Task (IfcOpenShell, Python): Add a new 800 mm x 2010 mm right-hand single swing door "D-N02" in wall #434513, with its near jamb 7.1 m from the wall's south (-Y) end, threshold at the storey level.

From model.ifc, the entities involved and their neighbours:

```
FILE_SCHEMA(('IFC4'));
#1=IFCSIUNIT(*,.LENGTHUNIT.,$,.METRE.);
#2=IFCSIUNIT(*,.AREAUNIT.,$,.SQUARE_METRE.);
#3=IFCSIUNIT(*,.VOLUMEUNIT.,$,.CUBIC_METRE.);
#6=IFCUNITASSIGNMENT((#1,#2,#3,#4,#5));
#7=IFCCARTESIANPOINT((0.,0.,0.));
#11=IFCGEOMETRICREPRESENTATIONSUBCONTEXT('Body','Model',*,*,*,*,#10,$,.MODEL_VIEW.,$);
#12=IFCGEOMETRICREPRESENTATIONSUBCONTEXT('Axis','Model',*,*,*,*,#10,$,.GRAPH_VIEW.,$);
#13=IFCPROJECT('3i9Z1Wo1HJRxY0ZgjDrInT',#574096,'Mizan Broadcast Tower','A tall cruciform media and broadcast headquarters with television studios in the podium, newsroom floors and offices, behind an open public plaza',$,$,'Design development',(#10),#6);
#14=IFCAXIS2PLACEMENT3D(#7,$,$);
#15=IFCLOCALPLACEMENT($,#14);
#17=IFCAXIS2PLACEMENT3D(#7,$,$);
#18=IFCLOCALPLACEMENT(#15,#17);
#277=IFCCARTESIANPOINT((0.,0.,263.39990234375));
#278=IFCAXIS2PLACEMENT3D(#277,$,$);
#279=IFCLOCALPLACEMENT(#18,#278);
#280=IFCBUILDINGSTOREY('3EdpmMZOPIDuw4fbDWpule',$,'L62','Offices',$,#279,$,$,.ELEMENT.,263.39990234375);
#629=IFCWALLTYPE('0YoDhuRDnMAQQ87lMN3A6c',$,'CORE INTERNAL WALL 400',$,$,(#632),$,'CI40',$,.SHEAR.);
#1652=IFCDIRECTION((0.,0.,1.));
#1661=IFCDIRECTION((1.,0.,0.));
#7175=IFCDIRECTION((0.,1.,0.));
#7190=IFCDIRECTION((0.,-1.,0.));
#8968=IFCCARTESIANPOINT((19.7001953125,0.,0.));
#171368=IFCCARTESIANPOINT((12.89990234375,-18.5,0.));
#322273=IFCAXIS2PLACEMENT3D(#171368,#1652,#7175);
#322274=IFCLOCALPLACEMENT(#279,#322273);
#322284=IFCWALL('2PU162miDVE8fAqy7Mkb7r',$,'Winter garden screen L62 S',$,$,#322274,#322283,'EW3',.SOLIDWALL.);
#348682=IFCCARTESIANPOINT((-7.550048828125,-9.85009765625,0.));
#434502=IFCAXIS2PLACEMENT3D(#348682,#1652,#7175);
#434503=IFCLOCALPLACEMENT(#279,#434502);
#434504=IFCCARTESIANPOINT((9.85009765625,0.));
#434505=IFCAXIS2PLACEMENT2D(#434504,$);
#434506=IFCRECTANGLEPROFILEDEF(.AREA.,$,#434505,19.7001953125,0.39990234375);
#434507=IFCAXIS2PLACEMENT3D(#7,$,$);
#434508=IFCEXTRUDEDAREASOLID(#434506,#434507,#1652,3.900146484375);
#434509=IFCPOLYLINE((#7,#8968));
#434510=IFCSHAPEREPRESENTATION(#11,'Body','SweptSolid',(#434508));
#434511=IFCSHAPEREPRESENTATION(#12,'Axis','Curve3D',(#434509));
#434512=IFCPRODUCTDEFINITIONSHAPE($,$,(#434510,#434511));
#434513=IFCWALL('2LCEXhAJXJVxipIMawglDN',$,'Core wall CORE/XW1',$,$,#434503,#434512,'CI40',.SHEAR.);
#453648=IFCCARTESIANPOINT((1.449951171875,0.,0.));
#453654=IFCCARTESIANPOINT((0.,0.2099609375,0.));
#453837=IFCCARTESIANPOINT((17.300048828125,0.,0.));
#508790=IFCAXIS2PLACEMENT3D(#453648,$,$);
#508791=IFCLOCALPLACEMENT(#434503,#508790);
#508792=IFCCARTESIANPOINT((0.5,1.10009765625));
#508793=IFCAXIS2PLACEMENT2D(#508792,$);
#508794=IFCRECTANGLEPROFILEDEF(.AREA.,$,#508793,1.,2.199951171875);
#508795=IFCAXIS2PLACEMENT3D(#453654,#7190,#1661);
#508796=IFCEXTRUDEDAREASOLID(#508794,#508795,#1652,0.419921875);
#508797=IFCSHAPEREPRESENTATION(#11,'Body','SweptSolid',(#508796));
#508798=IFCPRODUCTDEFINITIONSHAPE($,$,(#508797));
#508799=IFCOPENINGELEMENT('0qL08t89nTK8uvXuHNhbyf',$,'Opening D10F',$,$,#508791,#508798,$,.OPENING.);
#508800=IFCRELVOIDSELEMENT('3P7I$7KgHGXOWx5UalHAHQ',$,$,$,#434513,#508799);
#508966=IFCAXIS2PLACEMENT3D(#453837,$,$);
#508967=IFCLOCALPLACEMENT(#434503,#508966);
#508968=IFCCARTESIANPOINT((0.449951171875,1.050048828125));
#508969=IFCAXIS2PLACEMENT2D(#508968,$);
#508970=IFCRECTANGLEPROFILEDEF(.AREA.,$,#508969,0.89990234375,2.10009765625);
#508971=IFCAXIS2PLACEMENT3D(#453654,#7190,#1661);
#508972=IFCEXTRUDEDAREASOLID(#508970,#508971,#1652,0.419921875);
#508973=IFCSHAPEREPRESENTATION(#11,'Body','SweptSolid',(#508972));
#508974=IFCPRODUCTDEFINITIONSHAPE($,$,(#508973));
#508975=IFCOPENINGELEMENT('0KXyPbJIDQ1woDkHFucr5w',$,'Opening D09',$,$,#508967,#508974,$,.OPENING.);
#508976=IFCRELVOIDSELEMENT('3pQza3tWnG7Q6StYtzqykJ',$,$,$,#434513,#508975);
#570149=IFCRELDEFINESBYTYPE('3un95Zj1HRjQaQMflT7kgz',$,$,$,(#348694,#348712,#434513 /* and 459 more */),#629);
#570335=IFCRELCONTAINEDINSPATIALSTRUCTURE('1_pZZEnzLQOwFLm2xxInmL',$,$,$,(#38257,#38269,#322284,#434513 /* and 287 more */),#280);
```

```python
import numpy as np
import ifcopenshell
import ifcopenshell.api.feature
import ifcopenshell.api.geometry
import ifcopenshell.api.root
import ifcopenshell.api.spatial
import ifcopenshell.geom
import ifcopenshell.util.element
import ifcopenshell.util.placement
import ifcopenshell.util.representation
import ifcopenshell.util.shape
import ifcopenshell.util.unit

model = ifcopenshell.open("model.ifc")
unit_scale = ifcopenshell.util.unit.calculate_unit_scale(model)
settings = ifcopenshell.geom.settings()


def volume(element):
    """Net volume in cubic metres, openings subtracted."""
    shape = ifcopenshell.geom.create_shape(settings, element)
    return ifcopenshell.util.shape.get_volume(shape.geometry)


wall = model.by_guid("2LCEXhAJXJVxipIMawglDN")
storey = ifcopenshell.util.element.get_container(wall, ifc_class="IfcBuildingStorey")
context = ifcopenshell.util.representation.get_context(model, "Model", "Body", "MODEL_VIEW")
before = volume(wall)

width, height, from_end, sill = 0.8, 2.01, 7.1, 0.0  # metres

# The wall runs along its own X axis, and the end named is its -X end.
wall_shape = ifcopenshell.geom.create_shape(settings, wall)
x, y, z = ifcopenshell.util.shape.get_vertices(wall_shape.geometry).T
start = x.min() + from_end
face, thickness = float(y.min()), float(y.max() - y.min())
wall_matrix = ifcopenshell.util.placement.get_local_placement(wall.ObjectPlacement)
level = ifcopenshell.util.placement.get_local_placement(storey.ObjectPlacement)[2, 3]


def in_wall(x, y):
    """Placement at x, y metres in the wall's axes, at sill height."""
    matrix = wall_matrix.copy()
    matrix[:, 3] = wall_matrix @ np.array([x / unit_scale, y / unit_scale, 0.0, 1.0])
    matrix[2, 3] = level + sill / unit_scale
    return matrix


# Opening: a box that overshoots both wall faces by 50 mm.
opening = ifcopenshell.api.root.create_entity(model, ifc_class="IfcOpeningElement", predefined_type="OPENING")
box = ifcopenshell.api.geometry.add_wall_representation(
    model, context=context, length=width, height=height, thickness=thickness + 0.1
)
ifcopenshell.api.geometry.assign_representation(model, product=opening, representation=box)
ifcopenshell.api.geometry.edit_object_placement(model, product=opening, matrix=in_wall(start, face - 0.05), is_si=False)
ifcopenshell.api.feature.add_feature(model, feature=opening, element=wall)

door = ifcopenshell.api.root.create_entity(model, ifc_class="IfcDoor", name="D-N02", predefined_type="DOOR")
door.OverallWidth, door.OverallHeight = width / unit_scale, height / unit_scale
door.OperationType = "SINGLE_SWING_RIGHT"
body = ifcopenshell.api.geometry.add_door_representation(
    model,
    context=context,
    overall_width=door.OverallWidth,
    overall_height=door.OverallHeight,
    operation_type="SINGLE_SWING_RIGHT",
    lining_properties={"LiningDepth": thickness / unit_scale, "ThresholdDepth": thickness / unit_scale},
)
ifcopenshell.api.geometry.assign_representation(model, product=door, representation=body)
ifcopenshell.api.spatial.assign_container(model, products=[door], relating_structure=storey)
ifcopenshell.api.feature.add_filling(model, opening=opening, element=door)

# The lining spans the wall, so the door starts at the wall face.
ifcopenshell.api.geometry.edit_object_placement(model, product=door, matrix=in_wall(start, face), is_si=False)

after = volume(wall)

print(f"wall volume {before:.3f} -> {after:.3f} m3")

model.write("model-out.ifc")
```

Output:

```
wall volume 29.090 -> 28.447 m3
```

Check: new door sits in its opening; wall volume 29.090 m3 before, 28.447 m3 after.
